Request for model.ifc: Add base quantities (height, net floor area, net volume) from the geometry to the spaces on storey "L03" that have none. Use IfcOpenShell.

First a look at what the model holds.

```python
import ifcopenshell
import ifcopenshell.util.element
import ifcopenshell.util.unit

model = ifcopenshell.open("model.ifc")
print(model.schema)
for unit_type in ("LENGTHUNIT", "AREAUNIT", "VOLUMEUNIT"):
    print(unit_type, ifcopenshell.util.unit.calculate_unit_scale(model, unit_type))
storey = next(s for s in model.by_type("IfcBuildingStorey") if s.Name == "L03")
spaces = [e for e in ifcopenshell.util.element.get_decomposition(storey) if e.is_a("IfcSpace")]
for e in sorted(spaces, key=lambda e: e.id()):
    print(e.id(), e.is_a(), e.Name, list(ifcopenshell.util.element.get_psets(e, qtos_only=True)), sep=" | ")
```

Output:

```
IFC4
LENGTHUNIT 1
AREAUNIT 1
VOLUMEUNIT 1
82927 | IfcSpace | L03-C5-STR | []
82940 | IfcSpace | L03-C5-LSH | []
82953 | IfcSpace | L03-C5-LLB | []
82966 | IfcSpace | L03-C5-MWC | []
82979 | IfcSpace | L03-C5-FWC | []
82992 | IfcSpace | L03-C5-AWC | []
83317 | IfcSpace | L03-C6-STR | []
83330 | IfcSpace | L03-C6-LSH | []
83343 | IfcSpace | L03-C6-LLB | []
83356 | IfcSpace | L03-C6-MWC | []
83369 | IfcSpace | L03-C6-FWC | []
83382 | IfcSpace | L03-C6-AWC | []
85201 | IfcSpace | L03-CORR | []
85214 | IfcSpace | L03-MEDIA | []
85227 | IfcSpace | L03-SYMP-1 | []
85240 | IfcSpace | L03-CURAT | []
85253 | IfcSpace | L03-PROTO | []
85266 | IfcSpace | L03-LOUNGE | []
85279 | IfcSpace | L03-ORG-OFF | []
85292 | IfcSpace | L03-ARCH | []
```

```python
import ifcopenshell
import ifcopenshell.api.pset
import ifcopenshell.geom
import ifcopenshell.util.element
import ifcopenshell.util.shape
import ifcopenshell.util.unit

model = ifcopenshell.open("model.ifc")
unit_scale = ifcopenshell.util.unit.calculate_unit_scale(model)
area_scale = ifcopenshell.util.unit.calculate_unit_scale(model, "AREAUNIT")
volume_scale = ifcopenshell.util.unit.calculate_unit_scale(model, "VOLUMEUNIT")
settings = ifcopenshell.geom.settings()

storey = next(s for s in model.by_type("IfcBuildingStorey") if s.Name == "L03")
spaces = [e for e in ifcopenshell.util.element.get_decomposition(storey) if e.is_a("IfcSpace")]

for e in sorted(spaces, key=lambda e: e.id()):
    if ifcopenshell.util.element.get_psets(e, qtos_only=True, should_inherit=False):
        continue
    # Geometry comes back in metres, in the element's own axes.
    shape = ifcopenshell.geom.create_shape(settings, e)
    values = {
        "Height": ifcopenshell.util.shape.get_z(shape.geometry) / unit_scale,
        "NetFloorArea": ifcopenshell.util.shape.get_footprint_area(shape.geometry) / area_scale,
        "NetVolume": ifcopenshell.util.shape.get_volume(shape.geometry) / volume_scale,
    }
    qto = ifcopenshell.api.pset.add_qto(model, product=e, name="Qto_SpaceBaseQuantities")
    ifcopenshell.api.pset.edit_qto(model, qto=qto, properties=values)
    print(e.id(), {k: round(v, 3) for k, v in values.items()})

model.write("model-out.ifc")
```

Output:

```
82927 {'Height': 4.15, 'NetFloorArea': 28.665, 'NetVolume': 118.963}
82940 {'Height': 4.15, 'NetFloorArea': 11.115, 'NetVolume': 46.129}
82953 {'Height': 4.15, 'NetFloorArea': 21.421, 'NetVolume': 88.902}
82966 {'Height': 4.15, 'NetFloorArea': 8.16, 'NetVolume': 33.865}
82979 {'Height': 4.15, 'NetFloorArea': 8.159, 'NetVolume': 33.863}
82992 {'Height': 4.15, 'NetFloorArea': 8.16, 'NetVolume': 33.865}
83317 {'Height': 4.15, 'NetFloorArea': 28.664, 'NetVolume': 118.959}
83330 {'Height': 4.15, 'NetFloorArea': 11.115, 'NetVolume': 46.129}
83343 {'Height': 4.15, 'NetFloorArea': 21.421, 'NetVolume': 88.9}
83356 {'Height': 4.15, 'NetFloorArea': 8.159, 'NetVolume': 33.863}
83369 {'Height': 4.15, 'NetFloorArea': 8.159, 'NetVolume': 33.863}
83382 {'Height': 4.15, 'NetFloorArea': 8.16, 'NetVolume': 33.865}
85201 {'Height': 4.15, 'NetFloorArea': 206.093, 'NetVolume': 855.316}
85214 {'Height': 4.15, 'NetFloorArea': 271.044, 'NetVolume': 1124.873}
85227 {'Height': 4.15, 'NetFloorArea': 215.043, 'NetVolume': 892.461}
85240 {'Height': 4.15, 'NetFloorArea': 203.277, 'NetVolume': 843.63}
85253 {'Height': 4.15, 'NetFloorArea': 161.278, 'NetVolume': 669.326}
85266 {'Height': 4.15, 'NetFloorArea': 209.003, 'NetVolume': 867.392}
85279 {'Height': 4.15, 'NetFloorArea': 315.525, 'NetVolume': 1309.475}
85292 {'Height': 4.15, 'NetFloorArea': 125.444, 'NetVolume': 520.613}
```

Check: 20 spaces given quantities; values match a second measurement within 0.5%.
